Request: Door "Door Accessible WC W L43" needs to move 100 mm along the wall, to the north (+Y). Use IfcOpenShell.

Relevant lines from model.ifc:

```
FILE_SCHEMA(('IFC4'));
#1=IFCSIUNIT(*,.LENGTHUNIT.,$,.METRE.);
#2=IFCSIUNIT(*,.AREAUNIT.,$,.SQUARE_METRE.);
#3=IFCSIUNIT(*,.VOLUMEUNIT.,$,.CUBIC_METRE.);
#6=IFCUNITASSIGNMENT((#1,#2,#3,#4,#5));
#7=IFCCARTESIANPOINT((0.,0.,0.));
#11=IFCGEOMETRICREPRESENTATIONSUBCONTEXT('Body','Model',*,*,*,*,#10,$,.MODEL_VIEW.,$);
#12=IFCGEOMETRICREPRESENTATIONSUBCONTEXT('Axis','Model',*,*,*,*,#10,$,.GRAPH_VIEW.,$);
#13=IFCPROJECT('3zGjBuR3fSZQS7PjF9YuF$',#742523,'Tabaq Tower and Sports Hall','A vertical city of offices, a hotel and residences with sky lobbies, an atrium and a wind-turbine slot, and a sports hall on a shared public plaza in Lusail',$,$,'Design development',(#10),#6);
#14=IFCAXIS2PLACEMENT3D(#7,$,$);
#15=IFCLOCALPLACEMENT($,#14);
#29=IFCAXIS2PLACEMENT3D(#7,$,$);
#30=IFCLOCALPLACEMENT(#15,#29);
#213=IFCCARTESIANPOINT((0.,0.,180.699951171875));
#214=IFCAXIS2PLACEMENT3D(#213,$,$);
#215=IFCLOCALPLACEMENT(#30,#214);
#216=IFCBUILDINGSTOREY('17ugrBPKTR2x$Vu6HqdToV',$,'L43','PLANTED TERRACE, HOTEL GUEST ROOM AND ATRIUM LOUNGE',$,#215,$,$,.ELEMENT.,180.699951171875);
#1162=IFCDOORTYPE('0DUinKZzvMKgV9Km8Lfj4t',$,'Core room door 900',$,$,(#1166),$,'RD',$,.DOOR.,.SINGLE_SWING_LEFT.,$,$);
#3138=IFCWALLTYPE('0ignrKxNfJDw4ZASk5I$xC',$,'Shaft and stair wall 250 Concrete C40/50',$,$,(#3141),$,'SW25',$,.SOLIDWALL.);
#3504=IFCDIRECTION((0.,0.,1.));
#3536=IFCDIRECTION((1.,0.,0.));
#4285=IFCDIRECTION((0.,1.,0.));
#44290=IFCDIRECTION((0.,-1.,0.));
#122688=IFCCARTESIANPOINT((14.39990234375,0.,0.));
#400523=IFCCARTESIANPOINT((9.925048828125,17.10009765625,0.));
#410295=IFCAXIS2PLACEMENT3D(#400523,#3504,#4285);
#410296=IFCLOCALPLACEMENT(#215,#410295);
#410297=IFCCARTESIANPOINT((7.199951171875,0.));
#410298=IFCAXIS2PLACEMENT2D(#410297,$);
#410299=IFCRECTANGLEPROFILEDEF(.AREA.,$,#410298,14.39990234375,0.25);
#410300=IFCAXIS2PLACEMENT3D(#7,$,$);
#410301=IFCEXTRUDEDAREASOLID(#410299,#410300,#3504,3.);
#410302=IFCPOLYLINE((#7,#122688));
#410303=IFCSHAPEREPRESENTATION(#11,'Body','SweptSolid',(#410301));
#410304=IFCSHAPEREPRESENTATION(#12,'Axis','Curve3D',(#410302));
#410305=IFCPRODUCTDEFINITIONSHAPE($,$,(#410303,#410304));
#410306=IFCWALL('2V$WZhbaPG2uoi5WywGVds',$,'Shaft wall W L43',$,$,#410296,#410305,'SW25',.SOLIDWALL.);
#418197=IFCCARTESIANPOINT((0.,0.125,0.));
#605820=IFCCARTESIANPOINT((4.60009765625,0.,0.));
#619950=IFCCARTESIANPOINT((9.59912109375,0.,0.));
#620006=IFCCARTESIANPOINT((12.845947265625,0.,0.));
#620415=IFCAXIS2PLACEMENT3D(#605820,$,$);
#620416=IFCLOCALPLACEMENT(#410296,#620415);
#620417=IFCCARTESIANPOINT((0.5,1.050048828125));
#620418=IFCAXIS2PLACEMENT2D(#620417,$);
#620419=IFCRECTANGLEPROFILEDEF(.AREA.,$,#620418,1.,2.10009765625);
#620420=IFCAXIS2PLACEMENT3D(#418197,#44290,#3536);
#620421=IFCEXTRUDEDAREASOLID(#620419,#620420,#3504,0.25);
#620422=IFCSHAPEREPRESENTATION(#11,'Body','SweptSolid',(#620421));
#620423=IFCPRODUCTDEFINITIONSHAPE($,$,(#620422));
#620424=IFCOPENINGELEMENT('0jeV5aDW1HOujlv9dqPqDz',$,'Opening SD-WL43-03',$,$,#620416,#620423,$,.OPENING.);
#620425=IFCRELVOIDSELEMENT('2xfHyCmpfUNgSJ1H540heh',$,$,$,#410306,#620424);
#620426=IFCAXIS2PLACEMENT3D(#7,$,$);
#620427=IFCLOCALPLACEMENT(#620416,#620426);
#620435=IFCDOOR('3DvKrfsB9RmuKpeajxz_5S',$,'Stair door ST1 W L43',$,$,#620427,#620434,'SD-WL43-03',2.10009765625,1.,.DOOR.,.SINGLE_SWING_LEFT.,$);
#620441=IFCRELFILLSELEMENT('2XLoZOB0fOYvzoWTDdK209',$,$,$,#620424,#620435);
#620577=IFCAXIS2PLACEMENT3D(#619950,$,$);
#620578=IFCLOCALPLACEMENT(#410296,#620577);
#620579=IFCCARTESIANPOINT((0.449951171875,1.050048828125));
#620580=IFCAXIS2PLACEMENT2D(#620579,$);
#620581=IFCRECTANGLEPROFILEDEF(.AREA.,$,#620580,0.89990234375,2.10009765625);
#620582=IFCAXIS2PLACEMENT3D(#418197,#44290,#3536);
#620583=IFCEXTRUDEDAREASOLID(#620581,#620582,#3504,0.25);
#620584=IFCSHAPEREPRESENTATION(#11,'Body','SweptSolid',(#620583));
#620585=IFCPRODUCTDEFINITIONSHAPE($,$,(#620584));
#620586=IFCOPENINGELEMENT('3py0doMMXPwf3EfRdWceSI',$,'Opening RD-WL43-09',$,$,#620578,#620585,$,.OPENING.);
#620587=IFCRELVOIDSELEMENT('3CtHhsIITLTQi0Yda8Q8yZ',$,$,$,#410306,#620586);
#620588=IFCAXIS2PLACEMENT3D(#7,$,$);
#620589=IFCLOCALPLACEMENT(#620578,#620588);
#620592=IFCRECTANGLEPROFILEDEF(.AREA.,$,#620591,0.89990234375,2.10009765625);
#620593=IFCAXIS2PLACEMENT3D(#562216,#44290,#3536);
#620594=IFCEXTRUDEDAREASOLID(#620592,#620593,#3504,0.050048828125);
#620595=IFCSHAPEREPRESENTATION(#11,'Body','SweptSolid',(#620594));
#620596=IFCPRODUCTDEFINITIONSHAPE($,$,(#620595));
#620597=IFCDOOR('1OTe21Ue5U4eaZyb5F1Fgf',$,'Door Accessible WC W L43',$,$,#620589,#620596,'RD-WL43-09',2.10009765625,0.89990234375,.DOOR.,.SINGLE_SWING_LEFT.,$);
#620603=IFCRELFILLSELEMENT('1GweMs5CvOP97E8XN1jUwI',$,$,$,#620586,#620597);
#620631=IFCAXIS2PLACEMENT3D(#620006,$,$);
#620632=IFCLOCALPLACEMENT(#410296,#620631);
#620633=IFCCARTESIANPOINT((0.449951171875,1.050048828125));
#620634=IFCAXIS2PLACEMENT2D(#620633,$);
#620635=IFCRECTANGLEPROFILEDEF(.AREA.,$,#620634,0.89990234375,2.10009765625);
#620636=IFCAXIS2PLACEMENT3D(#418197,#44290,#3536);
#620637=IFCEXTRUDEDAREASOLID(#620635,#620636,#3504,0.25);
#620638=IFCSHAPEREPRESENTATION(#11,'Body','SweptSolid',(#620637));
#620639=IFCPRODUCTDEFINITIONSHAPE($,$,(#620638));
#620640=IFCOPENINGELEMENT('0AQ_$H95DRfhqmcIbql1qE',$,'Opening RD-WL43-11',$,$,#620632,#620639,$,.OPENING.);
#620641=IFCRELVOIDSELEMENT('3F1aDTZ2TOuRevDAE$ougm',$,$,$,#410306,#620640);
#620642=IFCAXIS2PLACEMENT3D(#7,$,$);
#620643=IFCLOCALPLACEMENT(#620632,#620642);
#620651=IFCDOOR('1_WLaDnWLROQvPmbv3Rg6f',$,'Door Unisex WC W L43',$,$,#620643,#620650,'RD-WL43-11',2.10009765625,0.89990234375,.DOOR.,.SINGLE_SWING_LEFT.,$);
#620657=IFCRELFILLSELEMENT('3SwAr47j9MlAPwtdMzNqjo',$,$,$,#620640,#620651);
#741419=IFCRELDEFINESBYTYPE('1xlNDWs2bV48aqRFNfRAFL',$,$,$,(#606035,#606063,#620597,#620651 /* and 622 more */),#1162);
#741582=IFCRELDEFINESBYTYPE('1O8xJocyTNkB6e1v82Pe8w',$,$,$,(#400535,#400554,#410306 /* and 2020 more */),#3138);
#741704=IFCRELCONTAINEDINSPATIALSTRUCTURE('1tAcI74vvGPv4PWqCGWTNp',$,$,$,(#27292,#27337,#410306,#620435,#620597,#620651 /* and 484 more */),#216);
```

```python
import ifcopenshell
import ifcopenshell.api.geometry
import ifcopenshell.util.placement
import ifcopenshell.util.unit

model = ifcopenshell.open("model.ifc")
unit_scale = ifcopenshell.util.unit.calculate_unit_scale(model)

door = model.by_guid("1OTe21Ue5U4eaZyb5F1Fgf")
opening = door.FillsVoids[0].RelatingOpeningElement
wall = opening.VoidsElements[0].RelatingBuildingElement

wall_matrix = ifcopenshell.util.placement.get_local_placement(wall.ObjectPlacement)
shift = wall_matrix[:3, 0] * 0.1 / unit_scale
before = ifcopenshell.util.placement.get_local_placement(door.ObjectPlacement)[:3, 3].copy()

# The door is placed relative to its opening, so it follows when the opening moves.
matrix = ifcopenshell.util.placement.get_local_placement(opening.ObjectPlacement)
matrix[:3, 3] += shift
ifcopenshell.api.geometry.edit_object_placement(
    model, product=opening, matrix=matrix, is_si=False, should_transform_children=True
)

after = ifcopenshell.util.placement.get_local_placement(door.ObjectPlacement)[:3, 3]
print("door moved by", (after - before).round(3) + 0.0)

model.write("model-out.ifc")
```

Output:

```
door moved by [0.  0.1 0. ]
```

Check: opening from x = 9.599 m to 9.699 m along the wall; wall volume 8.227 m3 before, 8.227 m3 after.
